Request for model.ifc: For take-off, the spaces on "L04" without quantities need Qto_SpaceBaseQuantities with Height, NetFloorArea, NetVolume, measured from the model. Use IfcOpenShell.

First a look at what the model holds.

```python
import ifcopenshell
import ifcopenshell.util.element
import ifcopenshell.util.unit

model = ifcopenshell.open("model.ifc")
print(model.schema)
for unit_type in ("LENGTHUNIT", "AREAUNIT", "VOLUMEUNIT"):
    print(unit_type, ifcopenshell.util.unit.calculate_unit_scale(model, unit_type))
storey = next(s for s in model.by_type("IfcBuildingStorey") if s.Name == "L04")
spaces = [e for e in ifcopenshell.util.element.get_decomposition(storey) if e.is_a("IfcSpace")]
for e in sorted(spaces, key=lambda e: e.id()):
    print(e.id(), e.is_a(), e.Name, list(ifcopenshell.util.element.get_psets(e, qtos_only=True)), sep=" | ")
```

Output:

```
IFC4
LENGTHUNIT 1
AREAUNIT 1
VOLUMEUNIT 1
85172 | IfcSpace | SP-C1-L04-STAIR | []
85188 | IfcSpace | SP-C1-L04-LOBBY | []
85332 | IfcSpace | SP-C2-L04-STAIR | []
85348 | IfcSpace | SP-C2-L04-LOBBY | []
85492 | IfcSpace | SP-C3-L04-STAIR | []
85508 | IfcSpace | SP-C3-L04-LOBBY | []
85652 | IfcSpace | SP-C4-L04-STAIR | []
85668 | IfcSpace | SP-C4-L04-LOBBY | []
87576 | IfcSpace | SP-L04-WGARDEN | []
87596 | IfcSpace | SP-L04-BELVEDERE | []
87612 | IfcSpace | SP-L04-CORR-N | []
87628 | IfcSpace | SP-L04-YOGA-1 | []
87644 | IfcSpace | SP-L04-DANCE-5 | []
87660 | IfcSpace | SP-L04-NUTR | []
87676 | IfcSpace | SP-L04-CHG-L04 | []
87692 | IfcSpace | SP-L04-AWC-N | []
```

```python
import ifcopenshell
import ifcopenshell.api.pset
import ifcopenshell.geom
import ifcopenshell.util.element
import ifcopenshell.util.shape
import ifcopenshell.util.unit

model = ifcopenshell.open("model.ifc")
unit_scale = ifcopenshell.util.unit.calculate_unit_scale(model)
area_scale = ifcopenshell.util.unit.calculate_unit_scale(model, "AREAUNIT")
volume_scale = ifcopenshell.util.unit.calculate_unit_scale(model, "VOLUMEUNIT")
settings = ifcopenshell.geom.settings()

storey = next(s for s in model.by_type("IfcBuildingStorey") if s.Name == "L04")
spaces = [e for e in ifcopenshell.util.element.get_decomposition(storey) if e.is_a("IfcSpace")]

for e in sorted(spaces, key=lambda e: e.id()):
    if ifcopenshell.util.element.get_psets(e, qtos_only=True, should_inherit=False):
        continue
    # Geometry comes back in metres, in the element's own axes.
    shape = ifcopenshell.geom.create_shape(settings, e)
    values = {
        "Height": ifcopenshell.util.shape.get_z(shape.geometry) / unit_scale,
        "NetFloorArea": ifcopenshell.util.shape.get_footprint_area(shape.geometry) / area_scale,
        "NetVolume": ifcopenshell.util.shape.get_volume(shape.geometry) / volume_scale,
    }
    qto = ifcopenshell.api.pset.add_qto(model, product=e, name="Qto_SpaceBaseQuantities")
    ifcopenshell.api.pset.edit_qto(model, qto=qto, properties=values)
    print(e.id(), {k: round(v, 3) for k, v in values.items()})

model.write("model-out.ifc")
```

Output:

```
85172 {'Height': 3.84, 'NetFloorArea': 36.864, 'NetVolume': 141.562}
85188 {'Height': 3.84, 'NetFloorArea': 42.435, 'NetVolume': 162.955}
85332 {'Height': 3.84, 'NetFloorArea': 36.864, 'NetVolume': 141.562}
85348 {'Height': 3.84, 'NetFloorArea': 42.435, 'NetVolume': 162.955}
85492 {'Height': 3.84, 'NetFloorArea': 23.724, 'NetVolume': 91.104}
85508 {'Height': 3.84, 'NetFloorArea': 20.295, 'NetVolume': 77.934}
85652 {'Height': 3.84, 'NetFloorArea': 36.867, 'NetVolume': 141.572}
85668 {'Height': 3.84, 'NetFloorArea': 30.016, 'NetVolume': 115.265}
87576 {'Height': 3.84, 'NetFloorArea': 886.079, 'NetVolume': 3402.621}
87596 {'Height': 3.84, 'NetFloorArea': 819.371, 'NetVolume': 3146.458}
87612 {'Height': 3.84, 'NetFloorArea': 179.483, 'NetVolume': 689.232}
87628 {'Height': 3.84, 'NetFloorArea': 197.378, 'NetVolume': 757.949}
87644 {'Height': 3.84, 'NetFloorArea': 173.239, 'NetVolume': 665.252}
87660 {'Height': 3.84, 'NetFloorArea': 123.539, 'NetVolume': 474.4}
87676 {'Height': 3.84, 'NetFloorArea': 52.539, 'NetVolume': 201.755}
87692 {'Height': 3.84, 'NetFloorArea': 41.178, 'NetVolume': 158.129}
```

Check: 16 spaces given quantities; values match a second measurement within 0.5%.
